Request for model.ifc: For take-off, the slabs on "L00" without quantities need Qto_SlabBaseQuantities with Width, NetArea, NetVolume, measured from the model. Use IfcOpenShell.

First a look at what the model holds.

```python
import ifcopenshell
import ifcopenshell.util.element
import ifcopenshell.util.unit

model = ifcopenshell.open("model.ifc")
print(model.schema)
for unit_type in ("LENGTHUNIT", "AREAUNIT", "VOLUMEUNIT"):
    print(unit_type, ifcopenshell.util.unit.calculate_unit_scale(model, unit_type))
storey = next(s for s in model.by_type("IfcBuildingStorey") if s.Name == "L00")
slabs = [e for e in ifcopenshell.util.element.get_decomposition(storey) if e.is_a("IfcSlab")]
for e in sorted(slabs, key=lambda e: e.id()):
    print(e.id(), e.is_a(), e.Name, list(ifcopenshell.util.element.get_psets(e, qtos_only=True)), sep=" | ")
```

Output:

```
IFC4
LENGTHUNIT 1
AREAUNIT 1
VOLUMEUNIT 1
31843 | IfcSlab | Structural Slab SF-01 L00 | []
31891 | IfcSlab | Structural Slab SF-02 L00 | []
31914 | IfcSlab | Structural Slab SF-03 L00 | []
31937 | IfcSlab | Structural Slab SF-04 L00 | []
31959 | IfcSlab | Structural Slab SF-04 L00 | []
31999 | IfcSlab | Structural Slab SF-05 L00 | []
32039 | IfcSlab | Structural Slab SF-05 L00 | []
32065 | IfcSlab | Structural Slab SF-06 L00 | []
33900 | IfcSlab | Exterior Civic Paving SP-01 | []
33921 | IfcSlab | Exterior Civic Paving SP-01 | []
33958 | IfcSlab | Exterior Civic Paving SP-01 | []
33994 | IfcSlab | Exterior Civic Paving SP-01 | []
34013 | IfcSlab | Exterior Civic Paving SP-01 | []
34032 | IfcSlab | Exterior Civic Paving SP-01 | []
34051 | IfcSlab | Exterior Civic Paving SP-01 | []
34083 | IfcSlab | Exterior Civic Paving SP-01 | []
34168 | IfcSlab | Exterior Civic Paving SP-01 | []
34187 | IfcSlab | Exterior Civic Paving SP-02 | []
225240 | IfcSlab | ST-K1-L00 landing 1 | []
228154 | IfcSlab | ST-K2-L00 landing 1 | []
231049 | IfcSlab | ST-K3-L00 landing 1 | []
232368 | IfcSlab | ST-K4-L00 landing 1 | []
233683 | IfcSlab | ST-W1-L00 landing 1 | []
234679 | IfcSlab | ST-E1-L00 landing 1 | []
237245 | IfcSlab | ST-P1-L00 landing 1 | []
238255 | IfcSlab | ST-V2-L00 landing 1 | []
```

```python
import ifcopenshell
import ifcopenshell.api.pset
import ifcopenshell.geom
import ifcopenshell.util.element
import ifcopenshell.util.shape
import ifcopenshell.util.unit

model = ifcopenshell.open("model.ifc")
unit_scale = ifcopenshell.util.unit.calculate_unit_scale(model)
area_scale = ifcopenshell.util.unit.calculate_unit_scale(model, "AREAUNIT")
volume_scale = ifcopenshell.util.unit.calculate_unit_scale(model, "VOLUMEUNIT")
settings = ifcopenshell.geom.settings()

storey = next(s for s in model.by_type("IfcBuildingStorey") if s.Name == "L00")
slabs = [e for e in ifcopenshell.util.element.get_decomposition(storey) if e.is_a("IfcSlab")]

for e in sorted(slabs, key=lambda e: e.id()):
    if ifcopenshell.util.element.get_psets(e, qtos_only=True, should_inherit=False):
        continue
    # Geometry comes back in metres, in the element's own axes.
    shape = ifcopenshell.geom.create_shape(settings, e)
    values = {
        "Width": ifcopenshell.util.shape.get_z(shape.geometry) / unit_scale,
        "NetArea": ifcopenshell.util.shape.get_footprint_area(shape.geometry) / area_scale,
        "NetVolume": ifcopenshell.util.shape.get_volume(shape.geometry) / volume_scale,
    }
    qto = ifcopenshell.api.pset.add_qto(model, product=e, name="Qto_SlabBaseQuantities")
    ifcopenshell.api.pset.edit_qto(model, qto=qto, properties=values)
    print(e.id(), {k: round(v, 3) for k, v in values.items()})

model.write("model_edited.ifc")
```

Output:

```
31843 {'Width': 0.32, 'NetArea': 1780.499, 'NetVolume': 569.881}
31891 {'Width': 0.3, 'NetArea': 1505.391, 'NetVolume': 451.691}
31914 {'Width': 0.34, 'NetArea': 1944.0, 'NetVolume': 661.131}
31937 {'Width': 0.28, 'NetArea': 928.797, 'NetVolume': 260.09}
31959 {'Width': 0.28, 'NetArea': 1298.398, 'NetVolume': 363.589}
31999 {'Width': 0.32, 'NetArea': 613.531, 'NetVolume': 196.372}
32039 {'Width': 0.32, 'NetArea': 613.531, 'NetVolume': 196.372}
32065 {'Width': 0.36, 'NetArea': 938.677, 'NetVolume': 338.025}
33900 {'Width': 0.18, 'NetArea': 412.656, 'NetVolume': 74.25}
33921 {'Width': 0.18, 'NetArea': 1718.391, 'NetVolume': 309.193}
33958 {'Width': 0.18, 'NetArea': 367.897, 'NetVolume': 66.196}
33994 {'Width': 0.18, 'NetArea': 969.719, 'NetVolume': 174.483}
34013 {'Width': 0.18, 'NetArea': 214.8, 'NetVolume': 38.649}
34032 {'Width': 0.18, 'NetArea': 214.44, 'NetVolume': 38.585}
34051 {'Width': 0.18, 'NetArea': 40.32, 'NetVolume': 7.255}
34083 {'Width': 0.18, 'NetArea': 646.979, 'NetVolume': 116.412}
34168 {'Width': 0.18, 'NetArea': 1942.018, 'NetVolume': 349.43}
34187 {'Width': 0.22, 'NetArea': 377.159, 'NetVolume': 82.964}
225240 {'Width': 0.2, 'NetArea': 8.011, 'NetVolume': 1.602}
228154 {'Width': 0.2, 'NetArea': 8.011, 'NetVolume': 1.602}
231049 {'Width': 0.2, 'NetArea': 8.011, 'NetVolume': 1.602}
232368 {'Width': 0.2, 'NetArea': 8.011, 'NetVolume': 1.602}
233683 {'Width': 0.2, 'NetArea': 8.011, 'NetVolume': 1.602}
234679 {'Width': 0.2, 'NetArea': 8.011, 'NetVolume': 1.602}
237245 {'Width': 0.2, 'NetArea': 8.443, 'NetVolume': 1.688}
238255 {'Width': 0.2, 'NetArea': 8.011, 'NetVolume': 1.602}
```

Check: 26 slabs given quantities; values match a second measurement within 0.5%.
